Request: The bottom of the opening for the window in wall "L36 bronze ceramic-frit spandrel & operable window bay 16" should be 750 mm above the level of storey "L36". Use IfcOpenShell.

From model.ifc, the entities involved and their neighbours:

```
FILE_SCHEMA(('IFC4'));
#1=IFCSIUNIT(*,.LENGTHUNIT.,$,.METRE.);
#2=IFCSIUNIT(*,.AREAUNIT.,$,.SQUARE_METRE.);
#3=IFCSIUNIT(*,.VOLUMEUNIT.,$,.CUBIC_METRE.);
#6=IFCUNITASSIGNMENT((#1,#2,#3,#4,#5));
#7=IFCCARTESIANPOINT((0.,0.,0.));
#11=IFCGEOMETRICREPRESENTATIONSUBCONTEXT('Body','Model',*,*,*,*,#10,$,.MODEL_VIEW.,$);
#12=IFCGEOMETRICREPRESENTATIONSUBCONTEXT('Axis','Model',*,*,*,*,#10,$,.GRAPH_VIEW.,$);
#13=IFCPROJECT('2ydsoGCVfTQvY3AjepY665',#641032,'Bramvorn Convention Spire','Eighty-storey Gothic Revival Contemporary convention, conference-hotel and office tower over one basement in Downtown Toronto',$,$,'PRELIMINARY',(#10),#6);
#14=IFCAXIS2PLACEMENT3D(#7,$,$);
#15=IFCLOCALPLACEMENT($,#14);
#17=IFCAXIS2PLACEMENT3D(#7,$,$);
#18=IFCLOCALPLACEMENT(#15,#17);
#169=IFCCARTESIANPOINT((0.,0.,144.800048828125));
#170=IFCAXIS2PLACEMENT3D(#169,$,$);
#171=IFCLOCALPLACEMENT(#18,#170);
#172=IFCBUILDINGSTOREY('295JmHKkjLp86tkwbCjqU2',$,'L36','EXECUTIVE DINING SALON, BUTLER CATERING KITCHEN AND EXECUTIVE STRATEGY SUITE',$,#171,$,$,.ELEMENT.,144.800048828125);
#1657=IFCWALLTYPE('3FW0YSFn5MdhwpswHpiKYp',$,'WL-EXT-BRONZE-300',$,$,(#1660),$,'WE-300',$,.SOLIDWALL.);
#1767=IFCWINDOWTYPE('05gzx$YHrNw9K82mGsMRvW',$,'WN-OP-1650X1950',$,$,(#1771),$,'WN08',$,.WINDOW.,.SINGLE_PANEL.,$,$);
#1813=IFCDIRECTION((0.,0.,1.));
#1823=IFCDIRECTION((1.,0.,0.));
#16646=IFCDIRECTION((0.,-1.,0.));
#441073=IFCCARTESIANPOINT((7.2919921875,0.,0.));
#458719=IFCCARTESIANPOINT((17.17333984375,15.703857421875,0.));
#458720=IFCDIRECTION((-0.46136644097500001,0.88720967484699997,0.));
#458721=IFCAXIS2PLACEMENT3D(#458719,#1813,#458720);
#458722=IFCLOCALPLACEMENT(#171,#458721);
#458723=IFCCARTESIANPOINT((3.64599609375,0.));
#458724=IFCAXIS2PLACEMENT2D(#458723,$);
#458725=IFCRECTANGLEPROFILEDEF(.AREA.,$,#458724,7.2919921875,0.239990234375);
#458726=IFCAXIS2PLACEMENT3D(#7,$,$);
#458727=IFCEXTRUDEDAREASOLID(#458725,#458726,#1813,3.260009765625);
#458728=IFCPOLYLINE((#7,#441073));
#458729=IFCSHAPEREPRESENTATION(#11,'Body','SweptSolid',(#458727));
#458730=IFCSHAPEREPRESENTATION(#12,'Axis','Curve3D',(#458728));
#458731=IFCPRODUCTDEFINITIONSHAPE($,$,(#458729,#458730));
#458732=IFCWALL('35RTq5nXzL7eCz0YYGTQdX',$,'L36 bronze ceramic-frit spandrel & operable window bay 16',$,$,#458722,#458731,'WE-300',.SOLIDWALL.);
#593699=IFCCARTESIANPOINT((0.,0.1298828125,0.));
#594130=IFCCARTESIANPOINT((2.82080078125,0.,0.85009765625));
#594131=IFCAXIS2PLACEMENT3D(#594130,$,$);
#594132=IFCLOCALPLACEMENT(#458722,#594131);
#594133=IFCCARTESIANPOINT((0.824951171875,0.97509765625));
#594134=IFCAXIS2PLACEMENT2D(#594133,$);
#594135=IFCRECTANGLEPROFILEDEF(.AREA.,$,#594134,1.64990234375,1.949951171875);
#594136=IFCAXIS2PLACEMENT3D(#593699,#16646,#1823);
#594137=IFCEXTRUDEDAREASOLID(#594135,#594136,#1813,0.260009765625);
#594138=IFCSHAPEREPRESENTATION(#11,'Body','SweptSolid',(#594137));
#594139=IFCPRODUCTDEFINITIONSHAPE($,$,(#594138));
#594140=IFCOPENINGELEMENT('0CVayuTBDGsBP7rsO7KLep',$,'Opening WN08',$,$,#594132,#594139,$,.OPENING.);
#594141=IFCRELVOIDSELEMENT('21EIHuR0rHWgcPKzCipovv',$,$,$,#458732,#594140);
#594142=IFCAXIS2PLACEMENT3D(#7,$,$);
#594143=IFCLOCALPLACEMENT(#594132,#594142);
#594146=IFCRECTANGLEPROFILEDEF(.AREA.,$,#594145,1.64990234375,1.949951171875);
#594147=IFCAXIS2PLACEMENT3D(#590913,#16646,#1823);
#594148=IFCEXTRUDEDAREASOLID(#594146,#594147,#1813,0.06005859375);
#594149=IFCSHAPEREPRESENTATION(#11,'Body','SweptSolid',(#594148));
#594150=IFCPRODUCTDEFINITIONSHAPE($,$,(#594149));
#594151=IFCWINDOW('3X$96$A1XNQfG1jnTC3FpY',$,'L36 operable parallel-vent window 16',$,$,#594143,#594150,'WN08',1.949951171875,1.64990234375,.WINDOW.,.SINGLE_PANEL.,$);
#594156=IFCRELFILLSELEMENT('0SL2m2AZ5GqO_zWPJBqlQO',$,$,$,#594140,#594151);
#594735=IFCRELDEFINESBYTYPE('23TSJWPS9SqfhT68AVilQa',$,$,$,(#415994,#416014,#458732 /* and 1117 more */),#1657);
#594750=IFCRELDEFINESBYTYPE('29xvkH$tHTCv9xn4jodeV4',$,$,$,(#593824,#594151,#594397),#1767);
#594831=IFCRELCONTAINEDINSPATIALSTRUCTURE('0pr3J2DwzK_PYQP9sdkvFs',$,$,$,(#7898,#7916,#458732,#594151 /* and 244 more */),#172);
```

```python
import numpy as np
import ifcopenshell
import ifcopenshell.api.geometry
import ifcopenshell.geom
import ifcopenshell.util.element
import ifcopenshell.util.placement
import ifcopenshell.util.shape
import ifcopenshell.util.unit

model = ifcopenshell.open("model.ifc")
unit_scale = ifcopenshell.util.unit.calculate_unit_scale(model)

window = model.by_id(594151)
opening = window.FillsVoids[0].RelatingOpeningElement
storey = ifcopenshell.util.element.get_container(window, ifc_class="IfcBuildingStorey")
level = ifcopenshell.util.placement.get_local_placement(storey.ObjectPlacement)[2, 3]

# The opening's origin need not be at the sill, so measure its lowest point.
shape = ifcopenshell.geom.create_shape(ifcopenshell.geom.settings(), opening)
bottom = ifcopenshell.util.shape.get_shape_bottom_elevation(shape, shape.geometry) / unit_scale
dz = level + 0.75 / unit_scale - bottom

shift = np.array([0.0, 0.0, dz])
# The window is placed relative to its opening, so it follows when the opening moves.
matrix = ifcopenshell.util.placement.get_local_placement(opening.ObjectPlacement)
matrix[:3, 3] += shift
ifcopenshell.api.geometry.edit_object_placement(
    model, product=opening, matrix=matrix, is_si=False, should_transform_children=True
)

print(f"moved by {dz * unit_scale:+.3f} m")

model.write("model_updated.ifc")
```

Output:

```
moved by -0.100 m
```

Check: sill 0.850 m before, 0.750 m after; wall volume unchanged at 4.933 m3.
